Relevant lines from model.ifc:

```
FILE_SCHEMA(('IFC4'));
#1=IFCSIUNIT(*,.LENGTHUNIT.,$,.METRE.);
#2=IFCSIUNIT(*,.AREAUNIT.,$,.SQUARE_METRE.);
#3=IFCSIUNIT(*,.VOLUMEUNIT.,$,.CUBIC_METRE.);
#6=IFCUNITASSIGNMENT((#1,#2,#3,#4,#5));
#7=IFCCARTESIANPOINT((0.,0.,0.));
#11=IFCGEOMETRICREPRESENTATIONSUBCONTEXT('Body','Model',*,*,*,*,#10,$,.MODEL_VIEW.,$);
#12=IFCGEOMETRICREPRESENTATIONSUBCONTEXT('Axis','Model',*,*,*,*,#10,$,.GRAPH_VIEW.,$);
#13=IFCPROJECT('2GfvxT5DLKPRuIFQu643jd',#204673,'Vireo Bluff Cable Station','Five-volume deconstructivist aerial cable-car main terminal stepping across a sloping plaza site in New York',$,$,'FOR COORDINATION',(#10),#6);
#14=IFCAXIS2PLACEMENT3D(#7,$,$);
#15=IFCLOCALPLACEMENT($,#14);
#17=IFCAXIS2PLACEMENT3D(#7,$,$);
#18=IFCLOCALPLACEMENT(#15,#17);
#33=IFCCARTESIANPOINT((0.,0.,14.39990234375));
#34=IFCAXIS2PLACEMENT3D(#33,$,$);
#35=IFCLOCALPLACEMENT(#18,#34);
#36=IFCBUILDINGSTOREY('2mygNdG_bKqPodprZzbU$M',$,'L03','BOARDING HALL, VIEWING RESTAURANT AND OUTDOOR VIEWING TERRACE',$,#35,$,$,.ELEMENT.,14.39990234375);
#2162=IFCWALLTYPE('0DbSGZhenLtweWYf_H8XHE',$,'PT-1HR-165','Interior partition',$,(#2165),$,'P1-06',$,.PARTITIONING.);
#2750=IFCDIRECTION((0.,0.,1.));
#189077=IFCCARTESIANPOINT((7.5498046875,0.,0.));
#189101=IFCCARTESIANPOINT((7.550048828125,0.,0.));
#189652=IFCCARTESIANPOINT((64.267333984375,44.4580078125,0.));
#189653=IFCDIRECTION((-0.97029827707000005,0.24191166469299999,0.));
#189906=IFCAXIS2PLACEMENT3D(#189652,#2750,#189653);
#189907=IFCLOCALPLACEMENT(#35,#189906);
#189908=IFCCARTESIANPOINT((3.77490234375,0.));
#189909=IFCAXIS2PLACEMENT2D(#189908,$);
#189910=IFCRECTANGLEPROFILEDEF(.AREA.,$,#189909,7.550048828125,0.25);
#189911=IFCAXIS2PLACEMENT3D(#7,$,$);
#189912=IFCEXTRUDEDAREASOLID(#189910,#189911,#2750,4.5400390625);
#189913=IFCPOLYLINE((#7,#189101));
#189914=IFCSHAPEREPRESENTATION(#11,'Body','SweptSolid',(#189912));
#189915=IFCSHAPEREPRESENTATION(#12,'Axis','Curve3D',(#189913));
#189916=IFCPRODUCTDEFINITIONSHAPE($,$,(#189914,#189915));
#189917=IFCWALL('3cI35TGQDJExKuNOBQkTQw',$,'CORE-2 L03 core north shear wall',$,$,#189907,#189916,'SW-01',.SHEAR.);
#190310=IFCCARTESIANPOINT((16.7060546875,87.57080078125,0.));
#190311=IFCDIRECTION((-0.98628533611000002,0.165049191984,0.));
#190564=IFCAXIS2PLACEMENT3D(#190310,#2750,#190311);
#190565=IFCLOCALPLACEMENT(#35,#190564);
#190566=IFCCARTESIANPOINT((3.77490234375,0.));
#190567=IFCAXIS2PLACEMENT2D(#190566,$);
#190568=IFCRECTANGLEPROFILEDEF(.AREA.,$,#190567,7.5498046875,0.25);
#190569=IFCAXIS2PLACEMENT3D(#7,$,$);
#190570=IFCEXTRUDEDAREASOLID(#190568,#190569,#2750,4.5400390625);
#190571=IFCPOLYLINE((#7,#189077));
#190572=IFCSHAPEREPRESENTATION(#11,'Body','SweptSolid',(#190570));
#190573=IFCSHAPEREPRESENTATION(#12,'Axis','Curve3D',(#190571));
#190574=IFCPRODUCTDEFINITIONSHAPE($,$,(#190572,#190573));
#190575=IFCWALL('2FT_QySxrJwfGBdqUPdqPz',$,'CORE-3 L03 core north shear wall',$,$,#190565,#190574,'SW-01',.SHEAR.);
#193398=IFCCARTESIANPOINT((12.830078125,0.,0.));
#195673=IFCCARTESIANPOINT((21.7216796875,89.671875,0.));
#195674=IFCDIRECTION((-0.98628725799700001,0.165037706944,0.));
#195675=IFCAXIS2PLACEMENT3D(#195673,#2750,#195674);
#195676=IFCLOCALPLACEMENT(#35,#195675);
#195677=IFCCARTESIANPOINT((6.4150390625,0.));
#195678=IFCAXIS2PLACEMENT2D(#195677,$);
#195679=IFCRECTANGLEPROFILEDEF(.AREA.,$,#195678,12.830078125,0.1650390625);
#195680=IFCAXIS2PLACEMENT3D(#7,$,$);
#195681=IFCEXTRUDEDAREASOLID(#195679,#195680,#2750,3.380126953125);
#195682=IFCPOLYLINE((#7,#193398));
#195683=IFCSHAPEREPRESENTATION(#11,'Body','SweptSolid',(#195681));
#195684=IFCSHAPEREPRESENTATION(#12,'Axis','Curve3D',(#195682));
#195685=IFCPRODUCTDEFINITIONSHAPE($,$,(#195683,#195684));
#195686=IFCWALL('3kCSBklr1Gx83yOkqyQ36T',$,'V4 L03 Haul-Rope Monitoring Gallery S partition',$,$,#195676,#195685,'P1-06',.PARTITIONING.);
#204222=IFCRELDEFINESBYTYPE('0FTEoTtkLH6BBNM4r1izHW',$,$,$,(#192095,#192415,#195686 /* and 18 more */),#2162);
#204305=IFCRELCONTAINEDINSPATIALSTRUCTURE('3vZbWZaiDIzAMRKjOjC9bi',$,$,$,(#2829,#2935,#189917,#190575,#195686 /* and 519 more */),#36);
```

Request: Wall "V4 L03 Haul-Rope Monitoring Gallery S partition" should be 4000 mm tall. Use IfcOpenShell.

```python
import ifcopenshell
import ifcopenshell.geom
import ifcopenshell.util.representation
import ifcopenshell.util.shape
import ifcopenshell.util.unit

model = ifcopenshell.open("model.ifc")
unit_scale = ifcopenshell.util.unit.calculate_unit_scale(model)
settings = ifcopenshell.geom.settings()


def volume(element):
    """Net volume in cubic metres, openings subtracted."""
    shape = ifcopenshell.geom.create_shape(settings, element)
    return ifcopenshell.util.shape.get_volume(shape.geometry)


wall = model.by_id(195686)
before = volume(wall)

body = ifcopenshell.util.representation.get_representation(wall, "Model", "Body")
solid = body.Items[0]
old_height = solid.Depth
solid.Depth = 4 / unit_scale
after = volume(wall)

print(f"height {old_height:g} -> {solid.Depth:g}, volume {before:.3f} -> {after:.3f} m3")

model.write("model_updated.ifc")
```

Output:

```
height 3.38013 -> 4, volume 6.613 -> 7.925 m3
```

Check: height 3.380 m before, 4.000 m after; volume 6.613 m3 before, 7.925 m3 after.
